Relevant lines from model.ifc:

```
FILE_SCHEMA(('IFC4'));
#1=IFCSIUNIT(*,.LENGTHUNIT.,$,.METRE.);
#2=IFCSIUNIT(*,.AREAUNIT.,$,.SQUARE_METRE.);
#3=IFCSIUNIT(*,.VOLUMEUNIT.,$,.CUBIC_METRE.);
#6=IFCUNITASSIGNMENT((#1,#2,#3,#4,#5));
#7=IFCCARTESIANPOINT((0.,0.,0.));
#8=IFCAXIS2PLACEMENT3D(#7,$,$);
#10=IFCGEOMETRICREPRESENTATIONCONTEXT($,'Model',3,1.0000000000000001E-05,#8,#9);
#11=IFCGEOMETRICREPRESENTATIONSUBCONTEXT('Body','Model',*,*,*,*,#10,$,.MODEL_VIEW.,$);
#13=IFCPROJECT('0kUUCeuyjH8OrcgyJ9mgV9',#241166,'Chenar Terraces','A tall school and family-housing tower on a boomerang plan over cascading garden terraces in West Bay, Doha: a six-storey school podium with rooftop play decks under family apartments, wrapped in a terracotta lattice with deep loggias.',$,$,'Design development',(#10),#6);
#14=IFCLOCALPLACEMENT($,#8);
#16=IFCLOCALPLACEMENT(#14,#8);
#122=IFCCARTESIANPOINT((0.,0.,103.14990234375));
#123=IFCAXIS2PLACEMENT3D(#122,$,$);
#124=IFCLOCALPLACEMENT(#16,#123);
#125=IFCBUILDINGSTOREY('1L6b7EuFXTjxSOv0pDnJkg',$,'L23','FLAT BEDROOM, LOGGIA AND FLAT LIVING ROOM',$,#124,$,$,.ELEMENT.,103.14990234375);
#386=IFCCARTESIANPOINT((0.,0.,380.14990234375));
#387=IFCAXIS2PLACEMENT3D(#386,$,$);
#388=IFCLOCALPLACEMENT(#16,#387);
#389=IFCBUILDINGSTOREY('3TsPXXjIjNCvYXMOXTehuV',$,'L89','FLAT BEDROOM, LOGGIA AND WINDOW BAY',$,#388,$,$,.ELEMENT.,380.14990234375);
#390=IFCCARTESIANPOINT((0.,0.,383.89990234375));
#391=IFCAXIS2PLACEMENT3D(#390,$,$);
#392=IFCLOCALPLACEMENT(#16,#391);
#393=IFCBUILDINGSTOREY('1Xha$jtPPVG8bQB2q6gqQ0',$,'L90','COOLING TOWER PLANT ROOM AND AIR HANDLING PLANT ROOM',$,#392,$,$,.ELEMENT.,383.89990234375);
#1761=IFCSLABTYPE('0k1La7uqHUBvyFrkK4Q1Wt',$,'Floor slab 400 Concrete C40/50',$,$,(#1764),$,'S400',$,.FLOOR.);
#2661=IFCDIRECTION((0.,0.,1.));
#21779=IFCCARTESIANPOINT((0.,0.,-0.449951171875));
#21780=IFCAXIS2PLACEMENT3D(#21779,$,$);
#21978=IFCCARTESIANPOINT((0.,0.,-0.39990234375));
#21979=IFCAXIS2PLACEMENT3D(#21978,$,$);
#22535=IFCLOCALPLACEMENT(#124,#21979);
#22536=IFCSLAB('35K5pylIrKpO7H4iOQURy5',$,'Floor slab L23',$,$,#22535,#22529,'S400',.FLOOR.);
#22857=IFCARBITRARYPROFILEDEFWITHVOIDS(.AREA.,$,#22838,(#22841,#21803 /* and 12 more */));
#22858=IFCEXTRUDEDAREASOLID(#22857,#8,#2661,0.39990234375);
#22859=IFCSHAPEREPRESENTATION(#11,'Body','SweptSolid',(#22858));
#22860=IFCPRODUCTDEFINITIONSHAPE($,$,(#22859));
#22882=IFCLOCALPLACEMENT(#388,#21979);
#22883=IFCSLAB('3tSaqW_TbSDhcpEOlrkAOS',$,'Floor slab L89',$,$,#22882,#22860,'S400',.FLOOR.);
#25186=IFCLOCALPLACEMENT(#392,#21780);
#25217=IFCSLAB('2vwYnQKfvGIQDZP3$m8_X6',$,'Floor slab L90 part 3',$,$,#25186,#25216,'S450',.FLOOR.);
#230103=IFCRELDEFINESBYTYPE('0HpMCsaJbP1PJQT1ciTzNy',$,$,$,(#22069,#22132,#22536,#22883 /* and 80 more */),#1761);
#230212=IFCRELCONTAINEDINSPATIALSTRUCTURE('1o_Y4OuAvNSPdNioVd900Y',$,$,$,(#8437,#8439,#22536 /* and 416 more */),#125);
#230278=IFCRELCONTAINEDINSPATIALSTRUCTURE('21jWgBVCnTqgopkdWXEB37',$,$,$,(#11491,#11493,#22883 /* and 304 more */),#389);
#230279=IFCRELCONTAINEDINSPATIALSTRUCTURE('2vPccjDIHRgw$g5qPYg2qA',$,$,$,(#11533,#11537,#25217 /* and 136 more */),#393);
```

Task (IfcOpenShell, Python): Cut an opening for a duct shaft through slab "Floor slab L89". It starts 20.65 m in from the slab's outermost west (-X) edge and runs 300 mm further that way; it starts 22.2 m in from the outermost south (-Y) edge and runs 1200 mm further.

```python
import numpy as np
import ifcopenshell
import ifcopenshell.api.feature
import ifcopenshell.api.geometry
import ifcopenshell.api.root
import ifcopenshell.geom
import ifcopenshell.util.placement
import ifcopenshell.util.representation
import ifcopenshell.util.shape
import ifcopenshell.util.unit

model = ifcopenshell.open("model.ifc")
unit_scale = ifcopenshell.util.unit.calculate_unit_scale(model)
settings = ifcopenshell.geom.settings()


def volume(element):
    """Net volume in cubic metres, openings subtracted."""
    shape = ifcopenshell.geom.create_shape(settings, element)
    return ifcopenshell.util.shape.get_volume(shape.geometry)


slab = model.by_guid("3tSaqW_TbSDhcpEOlrkAOS")
before = volume(slab)

# Extent in the slab's own axes, in metres. The edges named are its -X and -Y sides.
slab_shape = ifcopenshell.geom.create_shape(settings, slab)
vertices = ifcopenshell.util.shape.get_vertices(slab_shape.geometry)
x_min, y_min, bottom = vertices.min(axis=0)
top = vertices[:, 2].max()

opening = ifcopenshell.api.root.create_entity(model, ifc_class="IfcOpeningElement", name="Duct shaft opening", predefined_type="OPENING")
context = ifcopenshell.util.representation.get_context(model, "Model", "Body", "MODEL_VIEW")
width, depth = 0.3, 1.2
outline = [(0.0, 0.0), (width, 0.0), (width, depth), (0.0, depth), (0.0, 0.0)]
# Overshoot both faces by 50 mm so the cut is clean.
shape = ifcopenshell.api.geometry.add_slab_representation(
    model, context=context, depth=top - bottom + 0.1, polyline=outline
)
ifcopenshell.api.geometry.assign_representation(model, product=opening, representation=shape)

matrix = ifcopenshell.util.placement.get_local_placement(slab.ObjectPlacement)
matrix[:, 3] = matrix @ np.append(np.array([x_min + 20.65, y_min + 22.2, bottom - 0.05]) / unit_scale, 1.0)
ifcopenshell.api.geometry.edit_object_placement(model, product=opening, matrix=matrix, is_si=False)
ifcopenshell.api.feature.add_feature(model, feature=opening, element=slab)

after = volume(slab)

print(f"slab volume {before:.3f} -> {after:.3f} m3")

model.write("model_edited.ifc")
```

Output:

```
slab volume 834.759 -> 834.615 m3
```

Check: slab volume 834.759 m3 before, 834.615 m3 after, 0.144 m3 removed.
